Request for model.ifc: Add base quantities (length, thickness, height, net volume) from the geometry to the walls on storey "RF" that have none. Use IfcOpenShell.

First a look at what the model holds.

```python
import ifcopenshell
import ifcopenshell.util.element
import ifcopenshell.util.unit

model = ifcopenshell.open("model.ifc")
print(model.schema)
for unit_type in ("LENGTHUNIT", "AREAUNIT", "VOLUMEUNIT"):
    print(unit_type, ifcopenshell.util.unit.calculate_unit_scale(model, unit_type))
storey = next(s for s in model.by_type("IfcBuildingStorey") if s.Name == "RF")
walls = [e for e in ifcopenshell.util.element.get_decomposition(storey) if e.is_a("IfcWall")]
for e in sorted(walls, key=lambda e: e.id()):
    print(e.id(), e.is_a(), e.Name, list(ifcopenshell.util.element.get_psets(e, qtos_only=True)), sep=" | ")
```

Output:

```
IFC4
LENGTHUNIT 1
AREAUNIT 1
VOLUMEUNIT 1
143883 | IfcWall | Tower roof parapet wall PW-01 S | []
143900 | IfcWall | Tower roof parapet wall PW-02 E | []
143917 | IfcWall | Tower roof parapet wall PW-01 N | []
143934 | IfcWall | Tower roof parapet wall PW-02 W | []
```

```python
import ifcopenshell
import ifcopenshell.api.pset
import ifcopenshell.geom
import ifcopenshell.util.element
import ifcopenshell.util.shape
import ifcopenshell.util.unit

model = ifcopenshell.open("model.ifc")
unit_scale = ifcopenshell.util.unit.calculate_unit_scale(model)
volume_scale = ifcopenshell.util.unit.calculate_unit_scale(model, "VOLUMEUNIT")
settings = ifcopenshell.geom.settings()

storey = next(s for s in model.by_type("IfcBuildingStorey") if s.Name == "RF")
walls = [e for e in ifcopenshell.util.element.get_decomposition(storey) if e.is_a("IfcWall")]

for e in sorted(walls, key=lambda e: e.id()):
    if ifcopenshell.util.element.get_psets(e, qtos_only=True, should_inherit=False):
        continue
    # Geometry comes back in metres, in the element's own axes.
    shape = ifcopenshell.geom.create_shape(settings, e)
    values = {
        "Length": ifcopenshell.util.shape.get_x(shape.geometry) / unit_scale,
        "Width": ifcopenshell.util.shape.get_y(shape.geometry) / unit_scale,
        "Height": ifcopenshell.util.shape.get_z(shape.geometry) / unit_scale,
        "NetVolume": ifcopenshell.util.shape.get_volume(shape.geometry) / volume_scale,
    }
    qto = ifcopenshell.api.pset.add_qto(model, product=e, name="Qto_WallBaseQuantities")
    ifcopenshell.api.pset.edit_qto(model, qto=qto, properties=values)
    print(e.id(), {k: round(v, 3) for k, v in values.items()})

model.write("model_rev.ifc")
```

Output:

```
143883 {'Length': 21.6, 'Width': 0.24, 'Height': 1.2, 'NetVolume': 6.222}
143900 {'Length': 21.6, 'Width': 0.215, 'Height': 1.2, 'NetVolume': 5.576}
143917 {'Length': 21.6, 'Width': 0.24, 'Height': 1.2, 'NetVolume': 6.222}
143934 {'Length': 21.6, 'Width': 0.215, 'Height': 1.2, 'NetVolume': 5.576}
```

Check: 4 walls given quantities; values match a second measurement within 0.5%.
